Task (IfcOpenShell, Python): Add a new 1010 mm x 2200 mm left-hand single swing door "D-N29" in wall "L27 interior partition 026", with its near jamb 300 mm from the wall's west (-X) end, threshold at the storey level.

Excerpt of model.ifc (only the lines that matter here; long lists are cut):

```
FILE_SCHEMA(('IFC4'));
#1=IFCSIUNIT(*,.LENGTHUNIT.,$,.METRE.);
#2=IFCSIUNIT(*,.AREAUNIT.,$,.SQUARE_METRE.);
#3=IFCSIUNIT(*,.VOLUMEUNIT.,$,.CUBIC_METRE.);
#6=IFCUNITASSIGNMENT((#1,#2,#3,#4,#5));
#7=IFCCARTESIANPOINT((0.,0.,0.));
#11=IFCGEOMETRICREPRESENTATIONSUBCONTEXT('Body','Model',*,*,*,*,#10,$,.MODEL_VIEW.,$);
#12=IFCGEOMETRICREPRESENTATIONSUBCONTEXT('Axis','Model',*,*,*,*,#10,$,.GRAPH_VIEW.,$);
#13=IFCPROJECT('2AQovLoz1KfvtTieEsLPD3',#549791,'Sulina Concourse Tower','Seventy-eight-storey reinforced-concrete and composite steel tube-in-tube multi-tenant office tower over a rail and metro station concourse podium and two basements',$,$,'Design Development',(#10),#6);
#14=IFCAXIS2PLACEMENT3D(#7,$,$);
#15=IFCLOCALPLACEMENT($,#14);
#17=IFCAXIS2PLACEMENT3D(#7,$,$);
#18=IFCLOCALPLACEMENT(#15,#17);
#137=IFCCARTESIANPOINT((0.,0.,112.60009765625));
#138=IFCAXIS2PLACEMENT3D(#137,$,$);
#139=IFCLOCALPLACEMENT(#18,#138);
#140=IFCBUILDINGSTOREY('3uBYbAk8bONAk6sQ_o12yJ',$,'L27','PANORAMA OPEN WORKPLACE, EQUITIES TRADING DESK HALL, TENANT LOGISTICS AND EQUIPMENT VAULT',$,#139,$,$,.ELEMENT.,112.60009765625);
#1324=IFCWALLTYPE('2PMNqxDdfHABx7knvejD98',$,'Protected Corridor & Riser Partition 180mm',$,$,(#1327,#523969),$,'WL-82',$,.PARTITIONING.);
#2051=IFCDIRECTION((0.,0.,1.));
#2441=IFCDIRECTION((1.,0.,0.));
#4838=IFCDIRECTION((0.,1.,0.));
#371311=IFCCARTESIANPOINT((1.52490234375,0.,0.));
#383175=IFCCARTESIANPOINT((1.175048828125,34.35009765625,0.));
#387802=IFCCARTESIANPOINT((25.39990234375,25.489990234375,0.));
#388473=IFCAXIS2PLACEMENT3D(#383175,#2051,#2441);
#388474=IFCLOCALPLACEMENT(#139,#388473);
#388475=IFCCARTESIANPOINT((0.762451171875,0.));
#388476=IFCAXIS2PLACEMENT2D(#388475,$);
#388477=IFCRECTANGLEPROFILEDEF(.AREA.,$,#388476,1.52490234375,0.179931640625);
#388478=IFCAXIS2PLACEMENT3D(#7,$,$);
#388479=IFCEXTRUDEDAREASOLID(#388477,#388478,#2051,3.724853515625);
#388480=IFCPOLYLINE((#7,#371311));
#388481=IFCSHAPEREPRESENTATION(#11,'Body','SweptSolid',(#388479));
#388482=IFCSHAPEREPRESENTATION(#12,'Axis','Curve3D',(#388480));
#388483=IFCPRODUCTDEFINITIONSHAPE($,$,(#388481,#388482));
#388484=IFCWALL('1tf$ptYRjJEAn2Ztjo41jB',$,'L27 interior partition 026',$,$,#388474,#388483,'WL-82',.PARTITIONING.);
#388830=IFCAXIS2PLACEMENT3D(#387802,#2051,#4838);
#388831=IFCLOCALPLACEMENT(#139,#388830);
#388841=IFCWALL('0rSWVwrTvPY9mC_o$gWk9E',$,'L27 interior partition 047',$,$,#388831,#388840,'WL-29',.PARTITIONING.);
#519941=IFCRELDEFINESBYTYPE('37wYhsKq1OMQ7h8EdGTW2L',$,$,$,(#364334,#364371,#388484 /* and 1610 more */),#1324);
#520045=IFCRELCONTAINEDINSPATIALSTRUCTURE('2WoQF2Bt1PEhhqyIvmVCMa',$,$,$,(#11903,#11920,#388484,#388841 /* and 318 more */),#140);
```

```python
import numpy as np
import ifcopenshell
import ifcopenshell.api.feature
import ifcopenshell.api.geometry
import ifcopenshell.api.root
import ifcopenshell.api.spatial
import ifcopenshell.geom
import ifcopenshell.util.element
import ifcopenshell.util.placement
import ifcopenshell.util.representation
import ifcopenshell.util.shape
import ifcopenshell.util.unit

model = ifcopenshell.open("model.ifc")
unit_scale = ifcopenshell.util.unit.calculate_unit_scale(model)
settings = ifcopenshell.geom.settings()


def volume(element):
    """Net volume in cubic metres, openings subtracted."""
    shape = ifcopenshell.geom.create_shape(settings, element)
    return ifcopenshell.util.shape.get_volume(shape.geometry)


wall = model.by_guid("1tf$ptYRjJEAn2Ztjo41jB")
storey = ifcopenshell.util.element.get_container(wall, ifc_class="IfcBuildingStorey")
context = ifcopenshell.util.representation.get_context(model, "Model", "Body", "MODEL_VIEW")
before = volume(wall)

width, height, from_end, sill = 1.01, 2.2, 0.3, 0.0  # metres

# The wall runs along its own X axis, and the end named is its -X end.
wall_shape = ifcopenshell.geom.create_shape(settings, wall)
x, y, z = ifcopenshell.util.shape.get_vertices(wall_shape.geometry).T
start = x.min() + from_end
face, thickness = float(y.min()), float(y.max() - y.min())
wall_matrix = ifcopenshell.util.placement.get_local_placement(wall.ObjectPlacement)
level = ifcopenshell.util.placement.get_local_placement(storey.ObjectPlacement)[2, 3]


def in_wall(x, y):
    """Placement at x, y metres in the wall's axes, at sill height."""
    matrix = wall_matrix.copy()
    matrix[:, 3] = wall_matrix @ np.array([x / unit_scale, y / unit_scale, 0.0, 1.0])
    matrix[2, 3] = level + sill / unit_scale
    return matrix


# Opening: a box that overshoots both wall faces by 50 mm.
opening = ifcopenshell.api.root.create_entity(model, ifc_class="IfcOpeningElement", predefined_type="OPENING")
box = ifcopenshell.api.geometry.add_wall_representation(
    model, context=context, length=width, height=height, thickness=thickness + 0.1
)
ifcopenshell.api.geometry.assign_representation(model, product=opening, representation=box)
ifcopenshell.api.geometry.edit_object_placement(model, product=opening, matrix=in_wall(start, face - 0.05), is_si=False)
ifcopenshell.api.feature.add_feature(model, feature=opening, element=wall)

door = ifcopenshell.api.root.create_entity(model, ifc_class="IfcDoor", name="D-N29", predefined_type="DOOR")
door.OverallWidth, door.OverallHeight = width / unit_scale, height / unit_scale
door.OperationType = "SINGLE_SWING_LEFT"
body = ifcopenshell.api.geometry.add_door_representation(
    model,
    context=context,
    overall_width=door.OverallWidth,
    overall_height=door.OverallHeight,
    operation_type="SINGLE_SWING_LEFT",
    lining_properties={"LiningDepth": thickness / unit_scale, "ThresholdDepth": thickness / unit_scale},
)
ifcopenshell.api.geometry.assign_representation(model, product=door, representation=body)
ifcopenshell.api.spatial.assign_container(model, products=[door], relating_structure=storey)
ifcopenshell.api.feature.add_filling(model, opening=opening, element=door)

# The lining spans the wall, so the door starts at the wall face.
ifcopenshell.api.geometry.edit_object_placement(model, product=door, matrix=in_wall(start, face), is_si=False)

after = volume(wall)

print(f"wall volume {before:.3f} -> {after:.3f} m3")

model.write("model-out.ifc")
```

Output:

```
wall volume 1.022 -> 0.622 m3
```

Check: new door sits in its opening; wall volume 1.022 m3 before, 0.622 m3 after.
